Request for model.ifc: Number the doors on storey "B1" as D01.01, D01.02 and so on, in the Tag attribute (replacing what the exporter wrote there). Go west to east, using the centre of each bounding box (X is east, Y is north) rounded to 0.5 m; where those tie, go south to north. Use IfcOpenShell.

First a look at what the model holds.

```python
import ifcopenshell
import ifcopenshell.util.element
import ifcopenshell.util.placement

model = ifcopenshell.open("model.ifc")
print(model.schema)
storey = next(s for s in model.by_type("IfcBuildingStorey") if s.Name == "B1")
doors = [e for e in ifcopenshell.util.element.get_decomposition(storey) if e.is_a("IfcDoor")]
for e in sorted(doors, key=lambda e: e.id()):
    origin = ifcopenshell.util.placement.get_local_placement(e.ObjectPlacement)[:3, 3]
    print(e.id(), e.Tag, e.Name, origin.round(2) + 0.0, sep=" | ")
```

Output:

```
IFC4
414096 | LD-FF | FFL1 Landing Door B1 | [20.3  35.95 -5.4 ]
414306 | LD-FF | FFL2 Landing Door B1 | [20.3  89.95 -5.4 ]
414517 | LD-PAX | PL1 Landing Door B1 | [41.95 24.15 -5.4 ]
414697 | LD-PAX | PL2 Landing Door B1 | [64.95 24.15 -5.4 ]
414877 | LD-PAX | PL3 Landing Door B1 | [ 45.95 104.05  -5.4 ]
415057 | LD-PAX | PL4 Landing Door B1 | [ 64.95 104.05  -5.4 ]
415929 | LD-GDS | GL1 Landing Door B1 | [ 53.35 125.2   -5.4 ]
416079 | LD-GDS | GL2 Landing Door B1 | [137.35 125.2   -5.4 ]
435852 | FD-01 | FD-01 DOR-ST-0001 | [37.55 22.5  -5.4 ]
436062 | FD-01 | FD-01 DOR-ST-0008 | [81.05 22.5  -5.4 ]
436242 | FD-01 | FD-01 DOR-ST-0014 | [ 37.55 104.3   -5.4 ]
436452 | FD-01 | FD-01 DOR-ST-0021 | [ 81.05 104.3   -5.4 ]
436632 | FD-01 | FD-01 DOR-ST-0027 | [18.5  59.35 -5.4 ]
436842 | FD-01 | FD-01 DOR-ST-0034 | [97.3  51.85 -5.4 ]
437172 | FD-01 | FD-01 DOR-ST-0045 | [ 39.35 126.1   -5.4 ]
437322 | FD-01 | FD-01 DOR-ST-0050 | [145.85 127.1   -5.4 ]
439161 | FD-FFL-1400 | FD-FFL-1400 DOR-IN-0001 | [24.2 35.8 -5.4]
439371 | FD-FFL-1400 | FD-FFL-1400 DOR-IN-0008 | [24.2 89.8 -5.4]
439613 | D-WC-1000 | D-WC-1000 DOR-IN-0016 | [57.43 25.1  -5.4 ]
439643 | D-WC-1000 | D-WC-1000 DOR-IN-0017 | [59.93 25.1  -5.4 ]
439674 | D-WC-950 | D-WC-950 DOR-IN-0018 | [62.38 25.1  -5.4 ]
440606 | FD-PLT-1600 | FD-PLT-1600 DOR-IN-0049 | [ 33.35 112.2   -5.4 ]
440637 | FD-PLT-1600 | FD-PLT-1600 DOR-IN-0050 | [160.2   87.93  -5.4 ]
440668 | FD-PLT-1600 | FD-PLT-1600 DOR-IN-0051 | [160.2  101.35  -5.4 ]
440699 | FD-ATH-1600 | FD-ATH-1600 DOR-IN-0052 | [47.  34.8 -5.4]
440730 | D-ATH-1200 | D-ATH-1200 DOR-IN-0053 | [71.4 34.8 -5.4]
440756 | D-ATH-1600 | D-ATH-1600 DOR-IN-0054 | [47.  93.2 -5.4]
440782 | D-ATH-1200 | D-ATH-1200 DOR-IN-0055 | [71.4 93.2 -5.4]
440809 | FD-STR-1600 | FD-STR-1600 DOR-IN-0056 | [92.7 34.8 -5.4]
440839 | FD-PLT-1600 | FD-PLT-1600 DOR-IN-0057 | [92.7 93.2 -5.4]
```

```python
import ifcopenshell
import ifcopenshell.geom
import ifcopenshell.util.element
import ifcopenshell.util.shape

model = ifcopenshell.open("model.ifc")
settings = ifcopenshell.geom.settings()
settings.set("use-world-coords", True)


def centre(element):
    shape = ifcopenshell.geom.create_shape(settings, element)
    return ifcopenshell.util.shape.get_bbox_centroid(shape.geometry)


storey = next(s for s in model.by_type("IfcBuildingStorey") if s.Name == "B1")
doors = [e for e in ifcopenshell.util.element.get_decomposition(storey) if e.is_a("IfcDoor")]

# Insertion points can sit at a corner or the storey origin, so sort by the geometry (in metres).
centres = {e: centre(e) for e in doors}
doors.sort(key=lambda e: (round(centres[e][0] / 0.5), centres[e][1]))

for i, e in enumerate(doors, start=1):
    number = f"D01.{i:02d}"
    e.Tag = number
    print(e.id(), number)

model.write("model_edited.ifc")
```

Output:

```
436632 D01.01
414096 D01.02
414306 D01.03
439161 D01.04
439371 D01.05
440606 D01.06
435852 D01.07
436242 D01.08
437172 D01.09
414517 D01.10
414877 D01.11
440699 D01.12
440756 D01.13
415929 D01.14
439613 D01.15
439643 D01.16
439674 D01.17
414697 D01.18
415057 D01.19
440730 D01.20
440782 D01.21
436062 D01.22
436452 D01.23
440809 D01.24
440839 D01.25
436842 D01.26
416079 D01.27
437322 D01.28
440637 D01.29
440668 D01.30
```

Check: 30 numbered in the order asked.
